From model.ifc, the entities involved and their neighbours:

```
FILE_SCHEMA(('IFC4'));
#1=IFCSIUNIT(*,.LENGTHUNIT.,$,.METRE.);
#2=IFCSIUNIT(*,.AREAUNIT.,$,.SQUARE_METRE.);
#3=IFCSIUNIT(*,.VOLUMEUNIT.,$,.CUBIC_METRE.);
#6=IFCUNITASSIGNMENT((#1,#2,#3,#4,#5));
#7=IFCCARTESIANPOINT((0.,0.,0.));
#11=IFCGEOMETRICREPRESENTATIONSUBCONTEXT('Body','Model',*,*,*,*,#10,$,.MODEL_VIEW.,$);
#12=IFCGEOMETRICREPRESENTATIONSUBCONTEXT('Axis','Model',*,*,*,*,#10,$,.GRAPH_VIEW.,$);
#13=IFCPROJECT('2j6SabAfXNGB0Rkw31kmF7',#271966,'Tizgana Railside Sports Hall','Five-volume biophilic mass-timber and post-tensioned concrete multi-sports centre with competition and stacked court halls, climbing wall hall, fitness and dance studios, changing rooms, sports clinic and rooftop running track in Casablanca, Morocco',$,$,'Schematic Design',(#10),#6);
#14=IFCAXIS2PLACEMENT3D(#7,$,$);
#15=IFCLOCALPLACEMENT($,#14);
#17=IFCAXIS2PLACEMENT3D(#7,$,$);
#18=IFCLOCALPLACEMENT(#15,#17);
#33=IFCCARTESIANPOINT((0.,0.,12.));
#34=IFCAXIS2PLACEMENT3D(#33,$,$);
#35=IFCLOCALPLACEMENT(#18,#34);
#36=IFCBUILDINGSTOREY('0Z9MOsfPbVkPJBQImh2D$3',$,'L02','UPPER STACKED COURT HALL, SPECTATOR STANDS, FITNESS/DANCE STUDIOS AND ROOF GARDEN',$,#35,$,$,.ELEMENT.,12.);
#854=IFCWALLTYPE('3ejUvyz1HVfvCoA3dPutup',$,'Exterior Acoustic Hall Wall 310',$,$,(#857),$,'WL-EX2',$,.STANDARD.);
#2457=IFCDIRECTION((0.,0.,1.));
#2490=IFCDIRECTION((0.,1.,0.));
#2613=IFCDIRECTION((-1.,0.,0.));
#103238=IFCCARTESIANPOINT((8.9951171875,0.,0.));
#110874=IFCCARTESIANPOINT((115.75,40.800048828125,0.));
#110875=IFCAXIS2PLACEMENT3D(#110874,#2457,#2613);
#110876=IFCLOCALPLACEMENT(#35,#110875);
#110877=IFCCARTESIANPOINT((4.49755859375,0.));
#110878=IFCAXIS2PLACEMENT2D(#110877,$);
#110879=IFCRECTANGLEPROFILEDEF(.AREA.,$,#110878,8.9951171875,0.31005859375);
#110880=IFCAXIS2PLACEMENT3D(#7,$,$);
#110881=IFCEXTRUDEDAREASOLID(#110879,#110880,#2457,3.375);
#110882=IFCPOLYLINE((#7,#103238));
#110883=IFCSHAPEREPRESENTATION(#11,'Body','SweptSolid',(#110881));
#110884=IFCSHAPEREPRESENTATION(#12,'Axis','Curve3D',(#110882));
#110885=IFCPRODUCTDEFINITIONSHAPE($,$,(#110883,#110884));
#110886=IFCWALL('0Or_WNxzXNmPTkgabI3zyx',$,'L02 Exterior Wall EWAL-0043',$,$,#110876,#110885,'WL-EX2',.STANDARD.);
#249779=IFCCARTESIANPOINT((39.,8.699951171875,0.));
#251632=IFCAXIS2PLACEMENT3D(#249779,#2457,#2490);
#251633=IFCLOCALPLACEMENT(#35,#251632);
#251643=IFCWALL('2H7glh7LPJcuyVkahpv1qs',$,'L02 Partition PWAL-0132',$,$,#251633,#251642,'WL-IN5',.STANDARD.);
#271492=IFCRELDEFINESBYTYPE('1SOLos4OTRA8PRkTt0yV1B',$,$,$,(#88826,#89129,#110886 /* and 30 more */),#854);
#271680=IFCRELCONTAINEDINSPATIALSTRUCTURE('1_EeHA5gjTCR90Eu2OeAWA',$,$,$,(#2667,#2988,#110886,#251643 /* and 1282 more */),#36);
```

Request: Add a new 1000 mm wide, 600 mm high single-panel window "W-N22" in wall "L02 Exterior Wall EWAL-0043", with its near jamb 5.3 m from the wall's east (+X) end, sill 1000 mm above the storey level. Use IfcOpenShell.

```python
import numpy as np
import ifcopenshell
import ifcopenshell.api.feature
import ifcopenshell.api.geometry
import ifcopenshell.api.root
import ifcopenshell.api.spatial
import ifcopenshell.geom
import ifcopenshell.util.element
import ifcopenshell.util.placement
import ifcopenshell.util.representation
import ifcopenshell.util.shape
import ifcopenshell.util.unit

model = ifcopenshell.open("model.ifc")
unit_scale = ifcopenshell.util.unit.calculate_unit_scale(model)
settings = ifcopenshell.geom.settings()


def volume(element):
    """Net volume in cubic metres, openings subtracted."""
    shape = ifcopenshell.geom.create_shape(settings, element)
    return ifcopenshell.util.shape.get_volume(shape.geometry)


wall = model.by_id(110886)
storey = ifcopenshell.util.element.get_container(wall, ifc_class="IfcBuildingStorey")
context = ifcopenshell.util.representation.get_context(model, "Model", "Body", "MODEL_VIEW")
before = volume(wall)

width, height, from_end, sill = 1, 0.6, 5.3, 1  # metres

# The wall runs along its own X axis, and the end named is its -X end.
wall_shape = ifcopenshell.geom.create_shape(settings, wall)
x, y, z = ifcopenshell.util.shape.get_vertices(wall_shape.geometry).T
start = x.min() + from_end
face, thickness = float(y.min()), float(y.max() - y.min())
wall_matrix = ifcopenshell.util.placement.get_local_placement(wall.ObjectPlacement)
level = ifcopenshell.util.placement.get_local_placement(storey.ObjectPlacement)[2, 3]


def in_wall(x, y):
    """Placement at x, y metres in the wall's axes, at sill height."""
    matrix = wall_matrix.copy()
    matrix[:, 3] = wall_matrix @ np.array([x / unit_scale, y / unit_scale, 0.0, 1.0])
    matrix[2, 3] = level + sill / unit_scale
    return matrix


# Opening: a box that overshoots both wall faces by 50 mm.
opening = ifcopenshell.api.root.create_entity(model, ifc_class="IfcOpeningElement", predefined_type="OPENING")
box = ifcopenshell.api.geometry.add_wall_representation(
    model, context=context, length=width, height=height, thickness=thickness + 0.1
)
ifcopenshell.api.geometry.assign_representation(model, product=opening, representation=box)
ifcopenshell.api.geometry.edit_object_placement(model, product=opening, matrix=in_wall(start, face - 0.05), is_si=False)
ifcopenshell.api.feature.add_feature(model, feature=opening, element=wall)

window = ifcopenshell.api.root.create_entity(model, ifc_class="IfcWindow", name="W-N22", predefined_type="WINDOW")
window.OverallWidth, window.OverallHeight = width / unit_scale, height / unit_scale
window.PartitioningType = "SINGLE_PANEL"
body = ifcopenshell.api.geometry.add_window_representation(
    model,
    context=context,
    overall_width=window.OverallWidth,
    overall_height=window.OverallHeight,
    partition_type="SINGLE_PANEL",
)
ifcopenshell.api.geometry.assign_representation(model, product=window, representation=body)
ifcopenshell.api.spatial.assign_container(model, products=[window], relating_structure=storey)
ifcopenshell.api.feature.add_filling(model, opening=opening, element=window)

# Centre the window in the wall's thickness.
ifcopenshell.api.geometry.edit_object_placement(model, product=window, matrix=in_wall(start, face), is_si=False)
window_shape = ifcopenshell.geom.create_shape(settings, window)
depth = ifcopenshell.util.shape.get_vertices(window_shape.geometry)[:, 1]
offset = face + thickness / 2 - (depth.min() + depth.max()) / 2
ifcopenshell.api.geometry.edit_object_placement(model, product=window, matrix=in_wall(start, offset), is_si=False)

after = volume(wall)

print(f"wall volume {before:.3f} -> {after:.3f} m3")

model.write("model_edited.ifc")
```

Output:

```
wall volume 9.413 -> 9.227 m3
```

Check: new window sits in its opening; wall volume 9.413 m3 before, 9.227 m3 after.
